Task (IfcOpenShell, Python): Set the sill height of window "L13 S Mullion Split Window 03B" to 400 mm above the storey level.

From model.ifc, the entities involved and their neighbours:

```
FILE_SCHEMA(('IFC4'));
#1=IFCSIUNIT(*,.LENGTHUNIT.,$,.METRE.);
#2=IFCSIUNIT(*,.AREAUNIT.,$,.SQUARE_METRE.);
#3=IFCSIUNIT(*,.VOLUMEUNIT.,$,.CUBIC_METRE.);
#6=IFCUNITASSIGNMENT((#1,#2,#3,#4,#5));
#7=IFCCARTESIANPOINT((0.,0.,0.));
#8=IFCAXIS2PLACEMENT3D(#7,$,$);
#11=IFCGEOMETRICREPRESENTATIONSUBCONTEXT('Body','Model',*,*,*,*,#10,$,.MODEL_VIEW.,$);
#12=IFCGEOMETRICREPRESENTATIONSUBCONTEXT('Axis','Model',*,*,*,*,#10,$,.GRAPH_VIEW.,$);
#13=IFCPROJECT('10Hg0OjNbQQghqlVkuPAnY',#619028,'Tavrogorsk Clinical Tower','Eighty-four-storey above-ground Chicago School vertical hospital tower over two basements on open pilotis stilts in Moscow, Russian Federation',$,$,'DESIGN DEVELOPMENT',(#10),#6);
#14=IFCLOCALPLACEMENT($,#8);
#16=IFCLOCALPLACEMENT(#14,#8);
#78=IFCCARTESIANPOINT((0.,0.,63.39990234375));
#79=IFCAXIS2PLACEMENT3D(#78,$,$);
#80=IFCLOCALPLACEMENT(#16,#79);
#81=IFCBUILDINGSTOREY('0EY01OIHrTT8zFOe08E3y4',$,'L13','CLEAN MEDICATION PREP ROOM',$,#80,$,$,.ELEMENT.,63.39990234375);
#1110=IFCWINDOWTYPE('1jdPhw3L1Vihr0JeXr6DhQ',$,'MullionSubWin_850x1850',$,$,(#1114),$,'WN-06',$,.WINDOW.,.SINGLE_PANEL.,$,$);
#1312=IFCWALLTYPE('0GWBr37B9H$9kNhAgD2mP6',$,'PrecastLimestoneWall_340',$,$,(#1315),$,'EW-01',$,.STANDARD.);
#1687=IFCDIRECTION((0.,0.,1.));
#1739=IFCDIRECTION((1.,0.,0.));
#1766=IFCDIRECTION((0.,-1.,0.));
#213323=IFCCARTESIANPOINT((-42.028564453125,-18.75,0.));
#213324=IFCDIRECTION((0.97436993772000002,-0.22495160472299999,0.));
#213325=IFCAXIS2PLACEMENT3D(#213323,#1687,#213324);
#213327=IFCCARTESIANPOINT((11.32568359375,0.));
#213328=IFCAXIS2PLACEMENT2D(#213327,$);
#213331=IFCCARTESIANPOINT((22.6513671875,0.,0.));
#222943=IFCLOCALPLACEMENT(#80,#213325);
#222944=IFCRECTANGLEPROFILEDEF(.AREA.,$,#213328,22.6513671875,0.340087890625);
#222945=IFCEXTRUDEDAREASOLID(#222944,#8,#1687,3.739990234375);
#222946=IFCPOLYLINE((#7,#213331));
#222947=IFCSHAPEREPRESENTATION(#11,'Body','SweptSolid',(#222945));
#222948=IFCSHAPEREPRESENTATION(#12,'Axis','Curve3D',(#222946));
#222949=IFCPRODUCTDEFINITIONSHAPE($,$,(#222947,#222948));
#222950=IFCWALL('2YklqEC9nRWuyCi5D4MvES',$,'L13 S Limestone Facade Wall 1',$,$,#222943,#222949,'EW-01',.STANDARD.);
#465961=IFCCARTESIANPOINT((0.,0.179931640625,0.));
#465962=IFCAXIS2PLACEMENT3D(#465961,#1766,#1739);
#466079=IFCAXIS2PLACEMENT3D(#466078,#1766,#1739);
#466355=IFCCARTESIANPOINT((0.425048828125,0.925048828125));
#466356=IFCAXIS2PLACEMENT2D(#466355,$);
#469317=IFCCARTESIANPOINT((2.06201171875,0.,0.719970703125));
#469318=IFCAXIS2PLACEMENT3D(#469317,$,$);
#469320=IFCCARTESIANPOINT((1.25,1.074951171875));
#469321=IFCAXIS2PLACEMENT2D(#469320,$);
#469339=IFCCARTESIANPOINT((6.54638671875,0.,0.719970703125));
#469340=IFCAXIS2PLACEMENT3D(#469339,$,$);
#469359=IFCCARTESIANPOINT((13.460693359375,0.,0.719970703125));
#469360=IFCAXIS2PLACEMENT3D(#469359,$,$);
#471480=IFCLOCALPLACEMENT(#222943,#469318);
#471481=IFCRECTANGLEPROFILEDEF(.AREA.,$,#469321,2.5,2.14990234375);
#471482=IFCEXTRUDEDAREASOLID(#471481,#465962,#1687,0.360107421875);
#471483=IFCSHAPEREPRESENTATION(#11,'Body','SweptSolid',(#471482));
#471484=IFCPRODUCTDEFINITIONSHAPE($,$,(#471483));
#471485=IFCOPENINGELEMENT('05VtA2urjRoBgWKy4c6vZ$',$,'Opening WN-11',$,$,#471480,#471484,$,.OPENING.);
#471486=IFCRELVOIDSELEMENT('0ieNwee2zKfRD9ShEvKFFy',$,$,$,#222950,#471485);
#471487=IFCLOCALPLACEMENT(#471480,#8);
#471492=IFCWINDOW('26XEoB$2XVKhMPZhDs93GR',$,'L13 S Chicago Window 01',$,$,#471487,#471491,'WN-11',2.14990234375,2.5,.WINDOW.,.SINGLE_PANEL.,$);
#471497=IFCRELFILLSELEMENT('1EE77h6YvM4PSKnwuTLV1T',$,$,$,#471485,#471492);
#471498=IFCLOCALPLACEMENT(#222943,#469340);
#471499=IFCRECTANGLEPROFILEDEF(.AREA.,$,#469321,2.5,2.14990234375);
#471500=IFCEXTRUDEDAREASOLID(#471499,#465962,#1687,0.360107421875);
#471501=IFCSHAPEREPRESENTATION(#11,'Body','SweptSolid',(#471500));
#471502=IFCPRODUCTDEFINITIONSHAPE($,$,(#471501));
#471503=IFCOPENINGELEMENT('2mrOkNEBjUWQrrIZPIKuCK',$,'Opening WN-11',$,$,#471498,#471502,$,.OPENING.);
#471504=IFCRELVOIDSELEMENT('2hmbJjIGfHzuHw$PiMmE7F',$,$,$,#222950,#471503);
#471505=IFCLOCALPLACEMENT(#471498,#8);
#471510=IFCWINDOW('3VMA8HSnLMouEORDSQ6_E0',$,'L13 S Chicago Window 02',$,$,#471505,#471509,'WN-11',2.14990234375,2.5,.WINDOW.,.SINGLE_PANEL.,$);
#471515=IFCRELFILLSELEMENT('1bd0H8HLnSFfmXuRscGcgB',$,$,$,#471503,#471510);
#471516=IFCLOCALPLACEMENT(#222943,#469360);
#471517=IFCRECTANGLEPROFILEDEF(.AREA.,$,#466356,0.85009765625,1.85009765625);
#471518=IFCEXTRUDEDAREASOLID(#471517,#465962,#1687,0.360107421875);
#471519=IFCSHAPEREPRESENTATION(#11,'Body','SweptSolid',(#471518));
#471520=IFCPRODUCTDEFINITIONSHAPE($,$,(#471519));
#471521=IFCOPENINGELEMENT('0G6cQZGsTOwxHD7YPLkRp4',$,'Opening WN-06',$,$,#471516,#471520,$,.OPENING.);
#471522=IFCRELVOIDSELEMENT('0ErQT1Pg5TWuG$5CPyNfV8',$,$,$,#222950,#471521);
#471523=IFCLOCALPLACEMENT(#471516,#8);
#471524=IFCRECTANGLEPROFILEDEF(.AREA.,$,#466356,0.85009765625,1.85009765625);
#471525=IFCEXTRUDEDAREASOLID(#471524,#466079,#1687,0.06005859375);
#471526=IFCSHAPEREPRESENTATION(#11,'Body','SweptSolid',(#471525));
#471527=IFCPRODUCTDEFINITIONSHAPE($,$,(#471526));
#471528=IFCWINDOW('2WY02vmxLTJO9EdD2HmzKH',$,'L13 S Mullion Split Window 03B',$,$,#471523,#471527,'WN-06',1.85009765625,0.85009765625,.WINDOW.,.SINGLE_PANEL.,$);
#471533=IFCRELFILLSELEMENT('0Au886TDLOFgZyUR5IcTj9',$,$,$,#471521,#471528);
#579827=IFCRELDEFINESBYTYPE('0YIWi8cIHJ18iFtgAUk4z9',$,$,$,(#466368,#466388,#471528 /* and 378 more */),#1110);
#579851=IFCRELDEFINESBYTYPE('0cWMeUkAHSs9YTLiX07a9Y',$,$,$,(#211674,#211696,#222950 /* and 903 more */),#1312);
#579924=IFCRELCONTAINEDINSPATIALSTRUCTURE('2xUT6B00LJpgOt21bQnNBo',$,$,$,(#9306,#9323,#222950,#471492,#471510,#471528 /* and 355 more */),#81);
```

```python
import numpy as np
import ifcopenshell
import ifcopenshell.api.geometry
import ifcopenshell.geom
import ifcopenshell.util.element
import ifcopenshell.util.placement
import ifcopenshell.util.shape
import ifcopenshell.util.unit

model = ifcopenshell.open("model.ifc")
unit_scale = ifcopenshell.util.unit.calculate_unit_scale(model)

window = model.by_guid("2WY02vmxLTJO9EdD2HmzKH")
opening = window.FillsVoids[0].RelatingOpeningElement
storey = ifcopenshell.util.element.get_container(window, ifc_class="IfcBuildingStorey")
level = ifcopenshell.util.placement.get_local_placement(storey.ObjectPlacement)[2, 3]

# The opening's origin need not be at the sill, so measure its lowest point.
shape = ifcopenshell.geom.create_shape(ifcopenshell.geom.settings(), opening)
bottom = ifcopenshell.util.shape.get_shape_bottom_elevation(shape, shape.geometry) / unit_scale
dz = level + 0.4 - bottom

shift = np.array([0.0, 0.0, dz])
# The window is placed relative to its opening, so it follows when the opening moves.
matrix = ifcopenshell.util.placement.get_local_placement(opening.ObjectPlacement)
matrix[:3, 3] += shift
ifcopenshell.api.geometry.edit_object_placement(
    model, product=opening, matrix=matrix, is_si=False, should_transform_children=True
)

print(f"moved by {dz * unit_scale:+.3f} m")

model.write("model_updated.ifc")
```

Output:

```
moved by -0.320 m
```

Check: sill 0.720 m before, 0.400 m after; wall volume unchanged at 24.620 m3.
